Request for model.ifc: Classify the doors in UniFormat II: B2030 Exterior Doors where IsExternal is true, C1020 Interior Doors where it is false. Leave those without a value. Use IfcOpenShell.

First a look at what the model holds.

```python
import ifcopenshell
import ifcopenshell.util.element

model = ifcopenshell.open("model.ifc")
print(model.schema)
print("classifications:", [c.Name for c in model.by_type("IfcClassification")])
values = [ifcopenshell.util.element.get_pset(e, "Pset_DoorCommon", "IsExternal") for e in model.by_type("IfcDoor")]
for value in (True, False, None):
    print("IsExternal", value, values.count(value))
```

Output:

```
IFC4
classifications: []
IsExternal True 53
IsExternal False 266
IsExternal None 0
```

```python
import ifcopenshell
import ifcopenshell.api.classification
import ifcopenshell.util.element

model = ifcopenshell.open("model.ifc")

system = ifcopenshell.api.classification.add_classification(model, classification="UniFormat II")

doors = model.by_type("IfcDoor")
external = {e: ifcopenshell.util.element.get_pset(e, "Pset_DoorCommon", "IsExternal") for e in doors}
for flag, code, name in ((True, "B2030", "Exterior Doors"), (False, "C1020", "Interior Doors")):
    products = [e for e in doors if external[e] is flag]
    ifcopenshell.api.classification.add_reference(
        model, products=products, classification=system, identification=code, name=name
    )
    print(code, len(products))

model.write("model_rev.ifc")
```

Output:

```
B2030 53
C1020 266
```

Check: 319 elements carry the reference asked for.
